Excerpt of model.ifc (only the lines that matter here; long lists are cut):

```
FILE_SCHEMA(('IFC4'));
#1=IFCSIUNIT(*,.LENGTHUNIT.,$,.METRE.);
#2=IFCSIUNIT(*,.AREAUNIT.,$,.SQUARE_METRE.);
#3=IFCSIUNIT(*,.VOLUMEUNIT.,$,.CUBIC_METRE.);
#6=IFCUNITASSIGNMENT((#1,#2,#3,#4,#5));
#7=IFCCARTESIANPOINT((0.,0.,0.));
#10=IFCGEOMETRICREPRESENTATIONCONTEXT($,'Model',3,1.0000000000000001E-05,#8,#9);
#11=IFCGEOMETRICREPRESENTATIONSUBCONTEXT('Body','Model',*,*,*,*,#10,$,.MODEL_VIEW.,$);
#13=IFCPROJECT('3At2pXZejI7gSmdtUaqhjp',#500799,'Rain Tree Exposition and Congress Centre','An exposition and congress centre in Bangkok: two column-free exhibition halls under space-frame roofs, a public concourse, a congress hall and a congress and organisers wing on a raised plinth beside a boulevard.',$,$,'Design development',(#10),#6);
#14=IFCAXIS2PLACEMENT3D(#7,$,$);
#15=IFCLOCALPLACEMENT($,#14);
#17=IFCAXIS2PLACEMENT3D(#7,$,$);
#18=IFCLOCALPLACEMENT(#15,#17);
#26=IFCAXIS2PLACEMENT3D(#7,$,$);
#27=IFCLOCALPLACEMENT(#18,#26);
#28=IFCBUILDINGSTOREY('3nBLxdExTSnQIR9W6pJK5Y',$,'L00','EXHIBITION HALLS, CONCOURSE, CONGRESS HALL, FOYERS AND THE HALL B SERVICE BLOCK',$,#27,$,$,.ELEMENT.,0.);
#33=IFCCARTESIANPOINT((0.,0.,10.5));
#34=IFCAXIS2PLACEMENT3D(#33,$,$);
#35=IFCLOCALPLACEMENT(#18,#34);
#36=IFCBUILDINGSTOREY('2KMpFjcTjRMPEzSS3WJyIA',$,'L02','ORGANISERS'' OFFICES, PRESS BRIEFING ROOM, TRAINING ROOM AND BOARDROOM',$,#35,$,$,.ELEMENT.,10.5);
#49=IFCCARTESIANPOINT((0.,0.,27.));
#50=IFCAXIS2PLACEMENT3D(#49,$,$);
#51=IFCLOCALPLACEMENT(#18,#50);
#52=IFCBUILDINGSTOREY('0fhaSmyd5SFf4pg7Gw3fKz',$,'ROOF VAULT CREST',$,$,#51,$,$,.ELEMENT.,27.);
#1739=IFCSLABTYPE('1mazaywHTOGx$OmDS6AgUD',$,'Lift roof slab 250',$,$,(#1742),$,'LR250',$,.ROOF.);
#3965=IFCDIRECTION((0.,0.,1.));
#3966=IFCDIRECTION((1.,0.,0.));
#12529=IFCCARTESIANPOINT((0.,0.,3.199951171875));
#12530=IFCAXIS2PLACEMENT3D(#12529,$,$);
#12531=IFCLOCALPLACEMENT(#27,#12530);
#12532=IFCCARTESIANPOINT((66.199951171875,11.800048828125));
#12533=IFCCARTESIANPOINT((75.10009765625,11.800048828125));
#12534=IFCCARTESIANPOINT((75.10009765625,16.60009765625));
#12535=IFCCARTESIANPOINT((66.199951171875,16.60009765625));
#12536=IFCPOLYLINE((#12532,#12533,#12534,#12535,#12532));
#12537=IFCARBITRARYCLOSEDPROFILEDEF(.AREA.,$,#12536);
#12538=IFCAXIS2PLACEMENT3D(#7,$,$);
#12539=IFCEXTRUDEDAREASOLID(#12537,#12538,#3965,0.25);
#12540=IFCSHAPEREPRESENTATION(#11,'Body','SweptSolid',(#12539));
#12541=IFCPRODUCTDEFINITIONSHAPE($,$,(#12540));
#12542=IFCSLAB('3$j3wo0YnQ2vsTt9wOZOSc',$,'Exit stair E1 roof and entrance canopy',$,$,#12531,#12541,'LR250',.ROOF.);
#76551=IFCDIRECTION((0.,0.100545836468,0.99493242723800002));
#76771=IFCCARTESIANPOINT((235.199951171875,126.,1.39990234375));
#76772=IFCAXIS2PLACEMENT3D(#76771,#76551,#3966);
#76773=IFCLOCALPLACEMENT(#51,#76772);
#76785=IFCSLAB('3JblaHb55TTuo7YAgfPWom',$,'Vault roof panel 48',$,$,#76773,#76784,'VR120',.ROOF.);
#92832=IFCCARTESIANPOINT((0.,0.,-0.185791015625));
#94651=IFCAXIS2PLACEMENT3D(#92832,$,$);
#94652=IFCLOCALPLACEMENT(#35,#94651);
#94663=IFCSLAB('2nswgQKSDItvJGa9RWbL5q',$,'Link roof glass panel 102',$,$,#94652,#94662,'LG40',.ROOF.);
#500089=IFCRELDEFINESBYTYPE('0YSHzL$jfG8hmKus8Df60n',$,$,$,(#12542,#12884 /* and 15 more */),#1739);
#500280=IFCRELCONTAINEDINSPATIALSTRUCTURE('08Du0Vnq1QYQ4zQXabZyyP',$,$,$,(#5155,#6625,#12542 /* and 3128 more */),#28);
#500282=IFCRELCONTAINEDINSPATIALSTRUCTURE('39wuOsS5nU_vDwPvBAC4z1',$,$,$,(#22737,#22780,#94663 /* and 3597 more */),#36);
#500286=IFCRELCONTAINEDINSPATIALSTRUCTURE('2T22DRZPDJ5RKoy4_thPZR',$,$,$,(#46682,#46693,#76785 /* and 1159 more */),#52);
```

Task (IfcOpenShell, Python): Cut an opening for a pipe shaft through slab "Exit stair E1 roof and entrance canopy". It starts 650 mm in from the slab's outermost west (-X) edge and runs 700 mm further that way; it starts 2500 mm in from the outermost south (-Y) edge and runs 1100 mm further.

```python
import numpy as np
import ifcopenshell
import ifcopenshell.api.feature
import ifcopenshell.api.geometry
import ifcopenshell.api.root
import ifcopenshell.geom
import ifcopenshell.util.placement
import ifcopenshell.util.representation
import ifcopenshell.util.shape
import ifcopenshell.util.unit

model = ifcopenshell.open("model.ifc")
unit_scale = ifcopenshell.util.unit.calculate_unit_scale(model)
settings = ifcopenshell.geom.settings()


def volume(element):
    """Net volume in cubic metres, openings subtracted."""
    shape = ifcopenshell.geom.create_shape(settings, element)
    return ifcopenshell.util.shape.get_volume(shape.geometry)


slab = model.by_guid("3$j3wo0YnQ2vsTt9wOZOSc")
before = volume(slab)

# Extent in the slab's own axes, in metres. The edges named are its -X and -Y sides.
slab_shape = ifcopenshell.geom.create_shape(settings, slab)
vertices = ifcopenshell.util.shape.get_vertices(slab_shape.geometry)
x_min, y_min, bottom = vertices.min(axis=0)
top = vertices[:, 2].max()

opening = ifcopenshell.api.root.create_entity(model, ifc_class="IfcOpeningElement", name="Pipe shaft opening", predefined_type="OPENING")
context = ifcopenshell.util.representation.get_context(model, "Model", "Body", "MODEL_VIEW")
width, depth = 0.7, 1.1
outline = [(0.0, 0.0), (width, 0.0), (width, depth), (0.0, depth), (0.0, 0.0)]
# Overshoot both faces by 50 mm so the cut is clean.
shape = ifcopenshell.api.geometry.add_slab_representation(
    model, context=context, depth=top - bottom + 0.1, polyline=outline
)
ifcopenshell.api.geometry.assign_representation(model, product=opening, representation=shape)

matrix = ifcopenshell.util.placement.get_local_placement(slab.ObjectPlacement)
matrix[:, 3] = matrix @ np.append(np.array([x_min + 0.65, y_min + 2.5, bottom - 0.05]) / unit_scale, 1.0)
ifcopenshell.api.geometry.edit_object_placement(model, product=opening, matrix=matrix, is_si=False)
ifcopenshell.api.feature.add_feature(model, feature=opening, element=slab)

after = volume(slab)

print(f"slab volume {before:.3f} -> {after:.3f} m3")

model.write("model_updated.ifc")
```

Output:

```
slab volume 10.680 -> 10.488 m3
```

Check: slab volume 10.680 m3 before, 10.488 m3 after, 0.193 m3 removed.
